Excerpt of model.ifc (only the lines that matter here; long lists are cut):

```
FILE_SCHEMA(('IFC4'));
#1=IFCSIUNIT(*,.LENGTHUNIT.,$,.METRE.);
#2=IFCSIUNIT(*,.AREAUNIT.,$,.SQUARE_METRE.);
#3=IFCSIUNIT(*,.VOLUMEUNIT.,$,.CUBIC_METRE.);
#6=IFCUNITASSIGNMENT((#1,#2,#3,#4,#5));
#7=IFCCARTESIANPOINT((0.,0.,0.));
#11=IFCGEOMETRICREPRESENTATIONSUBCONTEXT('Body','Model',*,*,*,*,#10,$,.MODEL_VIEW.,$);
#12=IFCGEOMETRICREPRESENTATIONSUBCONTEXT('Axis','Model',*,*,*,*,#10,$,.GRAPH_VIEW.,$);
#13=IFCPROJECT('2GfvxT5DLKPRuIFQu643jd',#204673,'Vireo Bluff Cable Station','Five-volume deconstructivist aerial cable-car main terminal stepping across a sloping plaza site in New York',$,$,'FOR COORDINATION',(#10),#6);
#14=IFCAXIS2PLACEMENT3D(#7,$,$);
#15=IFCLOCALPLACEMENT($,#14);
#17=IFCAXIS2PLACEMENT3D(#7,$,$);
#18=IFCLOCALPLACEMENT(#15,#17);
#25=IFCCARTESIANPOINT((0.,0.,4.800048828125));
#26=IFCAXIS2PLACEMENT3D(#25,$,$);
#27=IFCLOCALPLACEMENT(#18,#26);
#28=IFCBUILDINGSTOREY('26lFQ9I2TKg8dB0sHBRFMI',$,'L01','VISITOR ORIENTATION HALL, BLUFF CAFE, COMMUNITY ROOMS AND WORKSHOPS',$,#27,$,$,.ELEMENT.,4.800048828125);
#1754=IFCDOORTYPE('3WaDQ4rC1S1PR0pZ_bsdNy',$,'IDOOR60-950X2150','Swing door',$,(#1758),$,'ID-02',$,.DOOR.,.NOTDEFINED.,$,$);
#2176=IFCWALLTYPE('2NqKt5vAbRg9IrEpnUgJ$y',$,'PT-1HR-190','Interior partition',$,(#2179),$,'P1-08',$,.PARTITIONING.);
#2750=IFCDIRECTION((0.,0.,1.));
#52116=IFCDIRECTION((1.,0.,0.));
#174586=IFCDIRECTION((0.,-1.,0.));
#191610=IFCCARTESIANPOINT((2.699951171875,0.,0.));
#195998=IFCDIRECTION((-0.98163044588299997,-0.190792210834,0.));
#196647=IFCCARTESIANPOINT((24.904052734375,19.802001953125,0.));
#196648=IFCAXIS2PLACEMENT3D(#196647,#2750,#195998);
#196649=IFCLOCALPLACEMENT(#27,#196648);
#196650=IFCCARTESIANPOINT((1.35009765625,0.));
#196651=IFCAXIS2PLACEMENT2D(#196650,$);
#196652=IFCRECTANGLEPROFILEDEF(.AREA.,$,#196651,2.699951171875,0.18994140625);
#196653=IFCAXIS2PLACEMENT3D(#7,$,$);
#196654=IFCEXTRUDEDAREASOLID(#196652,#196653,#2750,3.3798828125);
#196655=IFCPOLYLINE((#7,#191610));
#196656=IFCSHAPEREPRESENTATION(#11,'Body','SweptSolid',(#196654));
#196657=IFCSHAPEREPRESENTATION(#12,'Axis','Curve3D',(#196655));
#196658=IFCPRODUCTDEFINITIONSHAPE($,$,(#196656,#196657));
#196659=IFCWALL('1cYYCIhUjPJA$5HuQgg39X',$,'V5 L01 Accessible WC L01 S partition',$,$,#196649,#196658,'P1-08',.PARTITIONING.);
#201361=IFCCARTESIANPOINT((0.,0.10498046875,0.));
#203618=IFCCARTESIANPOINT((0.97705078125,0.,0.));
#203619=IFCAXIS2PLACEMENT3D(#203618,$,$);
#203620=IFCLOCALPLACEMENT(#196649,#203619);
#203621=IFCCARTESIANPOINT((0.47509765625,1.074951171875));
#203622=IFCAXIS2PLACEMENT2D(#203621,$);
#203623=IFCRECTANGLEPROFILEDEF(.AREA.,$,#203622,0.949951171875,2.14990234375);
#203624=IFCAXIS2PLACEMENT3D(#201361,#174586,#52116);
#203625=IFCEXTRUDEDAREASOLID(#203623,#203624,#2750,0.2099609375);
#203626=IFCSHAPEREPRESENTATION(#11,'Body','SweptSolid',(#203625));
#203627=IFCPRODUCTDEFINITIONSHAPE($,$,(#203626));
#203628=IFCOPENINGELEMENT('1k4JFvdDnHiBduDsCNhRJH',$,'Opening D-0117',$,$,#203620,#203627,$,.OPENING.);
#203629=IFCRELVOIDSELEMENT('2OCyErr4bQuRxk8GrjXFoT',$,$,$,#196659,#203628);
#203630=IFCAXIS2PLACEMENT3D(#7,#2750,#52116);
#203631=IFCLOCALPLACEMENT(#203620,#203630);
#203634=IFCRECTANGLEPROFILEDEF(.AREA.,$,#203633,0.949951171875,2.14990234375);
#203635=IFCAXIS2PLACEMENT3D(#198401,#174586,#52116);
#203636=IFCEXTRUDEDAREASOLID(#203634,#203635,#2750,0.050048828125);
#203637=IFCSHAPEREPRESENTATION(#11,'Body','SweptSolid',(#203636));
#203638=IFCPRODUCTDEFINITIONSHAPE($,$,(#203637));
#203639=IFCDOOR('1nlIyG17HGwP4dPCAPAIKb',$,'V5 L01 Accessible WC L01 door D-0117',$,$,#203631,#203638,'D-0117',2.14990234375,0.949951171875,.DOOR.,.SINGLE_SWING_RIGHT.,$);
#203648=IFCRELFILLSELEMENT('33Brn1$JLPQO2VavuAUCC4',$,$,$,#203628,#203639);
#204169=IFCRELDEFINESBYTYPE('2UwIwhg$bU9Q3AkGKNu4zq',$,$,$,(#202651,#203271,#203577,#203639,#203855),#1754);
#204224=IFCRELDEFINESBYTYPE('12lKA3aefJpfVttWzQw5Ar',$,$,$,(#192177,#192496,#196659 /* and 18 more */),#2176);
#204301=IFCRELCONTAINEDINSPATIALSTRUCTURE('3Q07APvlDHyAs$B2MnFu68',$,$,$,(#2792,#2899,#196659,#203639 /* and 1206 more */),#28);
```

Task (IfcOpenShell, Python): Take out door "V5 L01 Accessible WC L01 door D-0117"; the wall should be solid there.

```python
import ifcopenshell
import ifcopenshell.api.feature
import ifcopenshell.api.root
import ifcopenshell.geom
import ifcopenshell.util.shape

model = ifcopenshell.open("model.ifc")
settings = ifcopenshell.geom.settings()


def volume(element):
    """Net volume in cubic metres, openings subtracted."""
    shape = ifcopenshell.geom.create_shape(settings, element)
    return ifcopenshell.util.shape.get_volume(shape.geometry)


door = model.by_guid("1nlIyG17HGwP4dPCAPAIKb")
opening = door.FillsVoids[0].RelatingOpeningElement
wall = opening.VoidsElements[0].RelatingBuildingElement
before = volume(wall)

ifcopenshell.api.root.remove_product(model, product=door)
ifcopenshell.api.feature.remove_feature(model, feature=opening)

after = volume(wall)

print(f"wall volume {before:.3f} -> {after:.3f} m3")

model.write("model_updated.ifc")
```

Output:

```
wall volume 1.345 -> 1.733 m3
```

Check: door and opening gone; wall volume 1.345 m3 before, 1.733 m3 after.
